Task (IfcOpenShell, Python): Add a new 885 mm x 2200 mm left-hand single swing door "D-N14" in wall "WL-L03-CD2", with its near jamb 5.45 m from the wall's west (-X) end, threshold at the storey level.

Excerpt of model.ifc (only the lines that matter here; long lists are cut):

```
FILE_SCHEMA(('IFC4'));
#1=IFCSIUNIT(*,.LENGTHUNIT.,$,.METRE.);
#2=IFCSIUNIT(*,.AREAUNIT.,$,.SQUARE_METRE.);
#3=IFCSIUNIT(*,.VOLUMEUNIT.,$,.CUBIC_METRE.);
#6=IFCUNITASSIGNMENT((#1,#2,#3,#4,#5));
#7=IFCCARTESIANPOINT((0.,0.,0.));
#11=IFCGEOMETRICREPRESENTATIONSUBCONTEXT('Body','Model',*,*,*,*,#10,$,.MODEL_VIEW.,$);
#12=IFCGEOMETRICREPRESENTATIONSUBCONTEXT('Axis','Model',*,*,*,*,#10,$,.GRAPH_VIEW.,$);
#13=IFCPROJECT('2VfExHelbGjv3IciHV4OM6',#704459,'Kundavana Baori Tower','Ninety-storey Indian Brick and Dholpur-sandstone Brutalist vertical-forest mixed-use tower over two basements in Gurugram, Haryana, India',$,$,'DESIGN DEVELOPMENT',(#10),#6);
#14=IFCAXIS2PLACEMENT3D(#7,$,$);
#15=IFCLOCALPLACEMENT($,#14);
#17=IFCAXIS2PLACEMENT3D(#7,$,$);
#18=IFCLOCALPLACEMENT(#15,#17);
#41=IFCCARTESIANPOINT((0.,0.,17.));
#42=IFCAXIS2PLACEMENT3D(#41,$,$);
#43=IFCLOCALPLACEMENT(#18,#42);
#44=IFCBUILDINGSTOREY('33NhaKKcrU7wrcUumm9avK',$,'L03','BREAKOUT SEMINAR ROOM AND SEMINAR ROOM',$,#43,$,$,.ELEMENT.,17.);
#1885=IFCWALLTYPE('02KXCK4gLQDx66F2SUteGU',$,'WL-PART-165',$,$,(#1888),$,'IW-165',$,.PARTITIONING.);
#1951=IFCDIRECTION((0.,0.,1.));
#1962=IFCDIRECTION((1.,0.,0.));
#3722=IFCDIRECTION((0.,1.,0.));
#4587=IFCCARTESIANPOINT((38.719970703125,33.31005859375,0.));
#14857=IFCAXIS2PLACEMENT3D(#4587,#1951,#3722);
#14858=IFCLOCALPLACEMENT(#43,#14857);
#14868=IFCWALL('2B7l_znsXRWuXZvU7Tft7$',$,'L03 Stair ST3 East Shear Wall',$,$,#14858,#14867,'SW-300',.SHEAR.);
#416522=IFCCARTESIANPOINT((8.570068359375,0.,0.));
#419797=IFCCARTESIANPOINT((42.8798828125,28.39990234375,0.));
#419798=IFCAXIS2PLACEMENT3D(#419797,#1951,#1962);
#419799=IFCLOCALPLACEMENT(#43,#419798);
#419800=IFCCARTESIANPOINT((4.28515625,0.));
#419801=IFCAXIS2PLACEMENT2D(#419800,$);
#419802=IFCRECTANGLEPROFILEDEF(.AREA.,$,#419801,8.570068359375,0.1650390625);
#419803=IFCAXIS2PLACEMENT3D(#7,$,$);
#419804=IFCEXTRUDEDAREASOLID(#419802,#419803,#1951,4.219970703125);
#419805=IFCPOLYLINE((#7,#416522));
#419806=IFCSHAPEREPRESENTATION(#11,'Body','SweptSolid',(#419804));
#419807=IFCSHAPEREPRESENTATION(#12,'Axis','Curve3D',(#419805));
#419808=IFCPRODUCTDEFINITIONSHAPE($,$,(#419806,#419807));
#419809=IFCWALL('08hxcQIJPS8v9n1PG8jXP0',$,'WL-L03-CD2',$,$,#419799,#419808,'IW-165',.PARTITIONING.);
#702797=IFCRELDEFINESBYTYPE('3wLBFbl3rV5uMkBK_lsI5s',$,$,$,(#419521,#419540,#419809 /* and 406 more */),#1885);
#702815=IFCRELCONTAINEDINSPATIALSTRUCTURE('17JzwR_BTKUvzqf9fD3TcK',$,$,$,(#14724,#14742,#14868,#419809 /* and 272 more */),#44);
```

```python
import numpy as np
import ifcopenshell
import ifcopenshell.api.feature
import ifcopenshell.api.geometry
import ifcopenshell.api.root
import ifcopenshell.api.spatial
import ifcopenshell.geom
import ifcopenshell.util.element
import ifcopenshell.util.placement
import ifcopenshell.util.representation
import ifcopenshell.util.shape
import ifcopenshell.util.unit

model = ifcopenshell.open("model.ifc")
unit_scale = ifcopenshell.util.unit.calculate_unit_scale(model)
settings = ifcopenshell.geom.settings()


def volume(element):
    """Net volume in cubic metres, openings subtracted."""
    shape = ifcopenshell.geom.create_shape(settings, element)
    return ifcopenshell.util.shape.get_volume(shape.geometry)


wall = model.by_id(419809)
storey = ifcopenshell.util.element.get_container(wall, ifc_class="IfcBuildingStorey")
context = ifcopenshell.util.representation.get_context(model, "Model", "Body", "MODEL_VIEW")
before = volume(wall)

width, height, from_end, sill = 0.885, 2.2, 5.45, 0.0  # metres

# The wall runs along its own X axis, and the end named is its -X end.
wall_shape = ifcopenshell.geom.create_shape(settings, wall)
x, y, z = ifcopenshell.util.shape.get_vertices(wall_shape.geometry).T
start = x.min() + from_end
face, thickness = float(y.min()), float(y.max() - y.min())
wall_matrix = ifcopenshell.util.placement.get_local_placement(wall.ObjectPlacement)
level = ifcopenshell.util.placement.get_local_placement(storey.ObjectPlacement)[2, 3]


def in_wall(x, y):
    """Placement at x, y metres in the wall's axes, at sill height."""
    matrix = wall_matrix.copy()
    matrix[:, 3] = wall_matrix @ np.array([x / unit_scale, y / unit_scale, 0.0, 1.0])
    matrix[2, 3] = level + sill / unit_scale
    return matrix


# Opening: a box that overshoots both wall faces by 50 mm.
opening = ifcopenshell.api.root.create_entity(model, ifc_class="IfcOpeningElement", predefined_type="OPENING")
box = ifcopenshell.api.geometry.add_wall_representation(
    model, context=context, length=width, height=height, thickness=thickness + 0.1
)
ifcopenshell.api.geometry.assign_representation(model, product=opening, representation=box)
ifcopenshell.api.geometry.edit_object_placement(model, product=opening, matrix=in_wall(start, face - 0.05), is_si=False)
ifcopenshell.api.feature.add_feature(model, feature=opening, element=wall)

door = ifcopenshell.api.root.create_entity(model, ifc_class="IfcDoor", name="D-N14", predefined_type="DOOR")
door.OverallWidth, door.OverallHeight = width / unit_scale, height / unit_scale
door.OperationType = "SINGLE_SWING_LEFT"
body = ifcopenshell.api.geometry.add_door_representation(
    model,
    context=context,
    overall_width=door.OverallWidth,
    overall_height=door.OverallHeight,
    operation_type="SINGLE_SWING_LEFT",
    lining_properties={"LiningDepth": thickness / unit_scale, "ThresholdDepth": thickness / unit_scale},
)
ifcopenshell.api.geometry.assign_representation(model, product=door, representation=body)
ifcopenshell.api.spatial.assign_container(model, products=[door], relating_structure=storey)
ifcopenshell.api.feature.add_filling(model, opening=opening, element=door)

# The lining spans the wall, so the door starts at the wall face.
ifcopenshell.api.geometry.edit_object_placement(model, product=door, matrix=in_wall(start, face), is_si=False)

after = volume(wall)

print(f"wall volume {before:.3f} -> {after:.3f} m3")

model.write("model_rev.ifc")
```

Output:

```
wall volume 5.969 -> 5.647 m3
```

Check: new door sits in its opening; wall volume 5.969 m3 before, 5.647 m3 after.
